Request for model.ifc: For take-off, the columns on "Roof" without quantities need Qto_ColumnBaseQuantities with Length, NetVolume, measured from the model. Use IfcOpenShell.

First a look at what the model holds.

```python
import ifcopenshell
import ifcopenshell.util.element
import ifcopenshell.util.unit

model = ifcopenshell.open("model.ifc")
print(model.schema)
for unit_type in ("LENGTHUNIT", "AREAUNIT", "VOLUMEUNIT"):
    print(unit_type, ifcopenshell.util.unit.calculate_unit_scale(model, unit_type))
storey = next(s for s in model.by_type("IfcBuildingStorey") if s.Name == "Roof")
columns = [e for e in ifcopenshell.util.element.get_decomposition(storey) if e.is_a("IfcColumn")]
for e in sorted(columns, key=lambda e: e.id()):
    print(e.id(), e.is_a(), e.Name, list(ifcopenshell.util.element.get_psets(e, qtos_only=True)), sep=" | ")
```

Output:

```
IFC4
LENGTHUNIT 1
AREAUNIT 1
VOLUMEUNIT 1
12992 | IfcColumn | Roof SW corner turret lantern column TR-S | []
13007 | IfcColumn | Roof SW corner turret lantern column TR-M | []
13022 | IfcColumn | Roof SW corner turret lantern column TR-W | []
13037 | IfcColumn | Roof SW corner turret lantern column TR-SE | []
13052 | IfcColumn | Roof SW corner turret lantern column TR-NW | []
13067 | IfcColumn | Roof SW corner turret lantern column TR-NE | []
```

```python
import ifcopenshell
import ifcopenshell.api.pset
import ifcopenshell.geom
import ifcopenshell.util.element
import ifcopenshell.util.shape
import ifcopenshell.util.unit

model = ifcopenshell.open("model.ifc")
unit_scale = ifcopenshell.util.unit.calculate_unit_scale(model)
volume_scale = ifcopenshell.util.unit.calculate_unit_scale(model, "VOLUMEUNIT")
settings = ifcopenshell.geom.settings()

storey = next(s for s in model.by_type("IfcBuildingStorey") if s.Name == "Roof")
columns = [e for e in ifcopenshell.util.element.get_decomposition(storey) if e.is_a("IfcColumn")]

for e in sorted(columns, key=lambda e: e.id()):
    if ifcopenshell.util.element.get_psets(e, qtos_only=True, should_inherit=False):
        continue
    # Geometry comes back in metres, in the element's own axes.
    shape = ifcopenshell.geom.create_shape(settings, e)
    values = {
        "Length": ifcopenshell.util.shape.get_z(shape.geometry) / unit_scale,
        "NetVolume": ifcopenshell.util.shape.get_volume(shape.geometry) / volume_scale,
    }
    qto = ifcopenshell.api.pset.add_qto(model, product=e, name="Qto_ColumnBaseQuantities")
    ifcopenshell.api.pset.edit_qto(model, qto=qto, properties=values)
    print(e.id(), {k: round(v, 3) for k, v in values.items()})

model.write("model_edited.ifc")
```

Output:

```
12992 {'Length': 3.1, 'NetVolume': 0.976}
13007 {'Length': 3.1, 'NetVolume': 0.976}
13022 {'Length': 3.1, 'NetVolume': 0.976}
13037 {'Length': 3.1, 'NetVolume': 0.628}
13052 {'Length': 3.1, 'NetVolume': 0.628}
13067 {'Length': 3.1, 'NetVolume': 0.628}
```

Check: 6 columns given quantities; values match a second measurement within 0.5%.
